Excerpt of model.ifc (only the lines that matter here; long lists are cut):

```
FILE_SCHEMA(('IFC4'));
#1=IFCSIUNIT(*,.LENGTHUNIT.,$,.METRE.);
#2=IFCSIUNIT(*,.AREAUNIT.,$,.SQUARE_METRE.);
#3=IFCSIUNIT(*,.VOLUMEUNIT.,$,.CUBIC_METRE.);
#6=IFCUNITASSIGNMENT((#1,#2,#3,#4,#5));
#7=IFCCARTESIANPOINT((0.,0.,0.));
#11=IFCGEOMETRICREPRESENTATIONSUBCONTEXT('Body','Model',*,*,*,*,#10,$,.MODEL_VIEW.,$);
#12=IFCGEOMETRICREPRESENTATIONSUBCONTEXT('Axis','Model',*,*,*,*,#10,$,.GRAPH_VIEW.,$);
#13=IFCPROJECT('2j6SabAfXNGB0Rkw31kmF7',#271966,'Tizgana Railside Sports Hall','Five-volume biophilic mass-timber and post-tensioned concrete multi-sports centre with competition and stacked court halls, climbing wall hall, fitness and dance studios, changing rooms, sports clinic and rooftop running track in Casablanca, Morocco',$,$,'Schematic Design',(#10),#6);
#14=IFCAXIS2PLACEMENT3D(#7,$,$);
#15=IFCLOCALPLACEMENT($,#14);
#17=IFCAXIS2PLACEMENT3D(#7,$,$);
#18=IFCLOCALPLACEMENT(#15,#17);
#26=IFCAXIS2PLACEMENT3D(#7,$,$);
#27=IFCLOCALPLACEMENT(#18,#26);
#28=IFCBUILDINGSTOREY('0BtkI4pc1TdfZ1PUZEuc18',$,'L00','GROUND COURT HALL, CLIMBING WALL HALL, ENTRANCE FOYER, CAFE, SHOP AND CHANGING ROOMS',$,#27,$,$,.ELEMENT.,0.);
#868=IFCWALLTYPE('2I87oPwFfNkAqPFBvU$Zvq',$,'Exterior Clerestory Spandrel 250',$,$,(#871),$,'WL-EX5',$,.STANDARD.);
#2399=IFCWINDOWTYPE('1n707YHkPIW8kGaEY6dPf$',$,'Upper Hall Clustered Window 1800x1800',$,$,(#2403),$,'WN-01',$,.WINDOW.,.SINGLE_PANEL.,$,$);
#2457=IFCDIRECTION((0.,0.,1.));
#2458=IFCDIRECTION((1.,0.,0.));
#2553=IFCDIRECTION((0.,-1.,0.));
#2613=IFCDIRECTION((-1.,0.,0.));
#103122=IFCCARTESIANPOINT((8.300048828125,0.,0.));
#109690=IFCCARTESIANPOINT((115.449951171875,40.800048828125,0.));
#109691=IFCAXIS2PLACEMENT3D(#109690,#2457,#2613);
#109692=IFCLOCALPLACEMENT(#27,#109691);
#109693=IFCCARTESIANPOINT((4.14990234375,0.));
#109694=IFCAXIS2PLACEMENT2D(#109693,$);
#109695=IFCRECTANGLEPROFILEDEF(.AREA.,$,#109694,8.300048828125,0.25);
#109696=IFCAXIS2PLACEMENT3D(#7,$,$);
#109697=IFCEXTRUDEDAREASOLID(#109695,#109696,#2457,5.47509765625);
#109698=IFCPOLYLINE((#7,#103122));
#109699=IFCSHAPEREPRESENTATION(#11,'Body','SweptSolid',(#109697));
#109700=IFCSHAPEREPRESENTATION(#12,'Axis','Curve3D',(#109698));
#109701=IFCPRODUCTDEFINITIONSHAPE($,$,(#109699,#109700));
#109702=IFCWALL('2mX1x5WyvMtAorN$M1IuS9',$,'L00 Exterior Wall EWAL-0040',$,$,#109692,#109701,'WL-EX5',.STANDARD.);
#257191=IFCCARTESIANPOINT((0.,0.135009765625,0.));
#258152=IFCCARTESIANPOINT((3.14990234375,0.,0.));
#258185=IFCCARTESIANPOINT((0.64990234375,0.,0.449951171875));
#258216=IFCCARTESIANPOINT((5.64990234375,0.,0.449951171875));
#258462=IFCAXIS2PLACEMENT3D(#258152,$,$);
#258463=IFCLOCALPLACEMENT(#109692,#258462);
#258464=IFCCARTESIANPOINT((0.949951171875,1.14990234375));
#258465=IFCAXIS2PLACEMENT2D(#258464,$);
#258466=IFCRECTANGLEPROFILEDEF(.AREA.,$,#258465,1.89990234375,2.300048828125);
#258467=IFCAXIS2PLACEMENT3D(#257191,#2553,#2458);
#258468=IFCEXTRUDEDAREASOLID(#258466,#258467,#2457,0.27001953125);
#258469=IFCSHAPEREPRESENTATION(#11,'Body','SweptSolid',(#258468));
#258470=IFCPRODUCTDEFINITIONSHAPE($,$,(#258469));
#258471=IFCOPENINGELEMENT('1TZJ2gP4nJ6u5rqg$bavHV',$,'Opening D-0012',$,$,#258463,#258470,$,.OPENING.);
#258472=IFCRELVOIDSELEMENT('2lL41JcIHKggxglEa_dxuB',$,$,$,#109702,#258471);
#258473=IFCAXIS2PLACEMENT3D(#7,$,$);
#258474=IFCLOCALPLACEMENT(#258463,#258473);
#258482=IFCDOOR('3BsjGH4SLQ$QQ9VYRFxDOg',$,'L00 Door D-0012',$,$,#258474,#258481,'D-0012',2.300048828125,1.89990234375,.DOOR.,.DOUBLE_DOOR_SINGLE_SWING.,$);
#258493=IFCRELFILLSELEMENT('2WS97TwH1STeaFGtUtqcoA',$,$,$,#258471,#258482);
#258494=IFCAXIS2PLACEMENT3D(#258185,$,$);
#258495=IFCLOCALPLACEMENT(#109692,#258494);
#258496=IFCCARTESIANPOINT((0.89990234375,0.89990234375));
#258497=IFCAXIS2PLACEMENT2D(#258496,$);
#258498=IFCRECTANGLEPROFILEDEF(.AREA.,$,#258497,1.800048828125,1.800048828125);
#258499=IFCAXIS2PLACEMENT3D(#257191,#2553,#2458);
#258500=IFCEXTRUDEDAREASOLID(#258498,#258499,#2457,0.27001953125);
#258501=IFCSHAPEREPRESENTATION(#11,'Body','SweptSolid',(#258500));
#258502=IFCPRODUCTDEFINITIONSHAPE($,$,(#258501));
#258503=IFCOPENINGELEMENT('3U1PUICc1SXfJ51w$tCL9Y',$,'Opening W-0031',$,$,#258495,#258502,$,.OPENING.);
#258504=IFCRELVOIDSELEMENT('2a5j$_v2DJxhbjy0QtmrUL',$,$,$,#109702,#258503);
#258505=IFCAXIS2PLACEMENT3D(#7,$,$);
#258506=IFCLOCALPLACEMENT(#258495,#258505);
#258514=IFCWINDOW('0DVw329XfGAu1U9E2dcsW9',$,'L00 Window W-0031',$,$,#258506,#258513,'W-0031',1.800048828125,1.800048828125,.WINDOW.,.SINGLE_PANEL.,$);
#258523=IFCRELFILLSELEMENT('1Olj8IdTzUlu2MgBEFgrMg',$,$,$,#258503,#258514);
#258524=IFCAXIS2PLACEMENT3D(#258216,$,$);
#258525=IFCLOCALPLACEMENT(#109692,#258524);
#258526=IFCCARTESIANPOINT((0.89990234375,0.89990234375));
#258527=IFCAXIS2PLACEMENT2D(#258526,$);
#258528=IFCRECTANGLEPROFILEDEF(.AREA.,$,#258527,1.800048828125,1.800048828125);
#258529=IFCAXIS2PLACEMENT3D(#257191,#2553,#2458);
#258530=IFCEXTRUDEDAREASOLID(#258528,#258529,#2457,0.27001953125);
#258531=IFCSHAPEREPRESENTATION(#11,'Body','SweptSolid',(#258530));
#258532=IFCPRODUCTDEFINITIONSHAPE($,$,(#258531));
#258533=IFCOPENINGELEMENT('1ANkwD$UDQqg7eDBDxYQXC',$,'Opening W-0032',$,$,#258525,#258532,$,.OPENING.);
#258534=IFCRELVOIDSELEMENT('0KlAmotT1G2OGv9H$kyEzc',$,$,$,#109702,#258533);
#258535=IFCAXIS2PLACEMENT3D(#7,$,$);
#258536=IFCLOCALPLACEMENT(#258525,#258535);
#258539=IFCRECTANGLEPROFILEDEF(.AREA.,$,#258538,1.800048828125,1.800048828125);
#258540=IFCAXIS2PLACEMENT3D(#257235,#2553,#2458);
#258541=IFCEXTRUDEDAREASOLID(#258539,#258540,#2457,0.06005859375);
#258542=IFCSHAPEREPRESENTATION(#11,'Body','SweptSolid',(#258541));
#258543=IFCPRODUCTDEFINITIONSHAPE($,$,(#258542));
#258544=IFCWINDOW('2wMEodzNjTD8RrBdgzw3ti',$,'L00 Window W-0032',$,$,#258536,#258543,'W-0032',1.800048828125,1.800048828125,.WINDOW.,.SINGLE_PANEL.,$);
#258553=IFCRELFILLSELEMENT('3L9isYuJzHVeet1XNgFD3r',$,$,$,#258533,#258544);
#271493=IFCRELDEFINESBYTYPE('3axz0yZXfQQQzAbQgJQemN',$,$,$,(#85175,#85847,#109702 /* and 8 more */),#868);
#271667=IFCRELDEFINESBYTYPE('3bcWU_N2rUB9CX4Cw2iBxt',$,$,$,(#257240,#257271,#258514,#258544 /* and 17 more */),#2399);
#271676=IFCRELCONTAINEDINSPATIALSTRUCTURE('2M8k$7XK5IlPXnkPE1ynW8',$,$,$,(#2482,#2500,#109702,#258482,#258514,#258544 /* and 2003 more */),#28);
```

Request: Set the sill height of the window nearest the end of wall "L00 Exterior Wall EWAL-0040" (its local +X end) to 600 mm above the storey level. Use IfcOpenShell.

```python
import numpy as np
import ifcopenshell
import ifcopenshell.api.geometry
import ifcopenshell.geom
import ifcopenshell.util.element
import ifcopenshell.util.placement
import ifcopenshell.util.shape
import ifcopenshell.util.unit

model = ifcopenshell.open("model.ifc")
unit_scale = ifcopenshell.util.unit.calculate_unit_scale(model)

window = model.by_guid("2wMEodzNjTD8RrBdgzw3ti")
opening = window.FillsVoids[0].RelatingOpeningElement
storey = ifcopenshell.util.element.get_container(window, ifc_class="IfcBuildingStorey")
level = ifcopenshell.util.placement.get_local_placement(storey.ObjectPlacement)[2, 3]

# The opening's origin need not be at the sill, so measure its lowest point.
shape = ifcopenshell.geom.create_shape(ifcopenshell.geom.settings(), opening)
bottom = ifcopenshell.util.shape.get_shape_bottom_elevation(shape, shape.geometry) / unit_scale
dz = level + 0.6 / unit_scale - bottom

shift = np.array([0.0, 0.0, dz])
# The window is placed relative to its opening, so it follows when the opening moves.
matrix = ifcopenshell.util.placement.get_local_placement(opening.ObjectPlacement)
matrix[:3, 3] += shift
ifcopenshell.api.geometry.edit_object_placement(
    model, product=opening, matrix=matrix, is_si=False, should_transform_children=True
)

print(f"moved by {dz * unit_scale:+.3f} m")

model.write("model_rev.ifc")
```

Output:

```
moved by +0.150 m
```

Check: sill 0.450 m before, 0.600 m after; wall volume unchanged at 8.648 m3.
